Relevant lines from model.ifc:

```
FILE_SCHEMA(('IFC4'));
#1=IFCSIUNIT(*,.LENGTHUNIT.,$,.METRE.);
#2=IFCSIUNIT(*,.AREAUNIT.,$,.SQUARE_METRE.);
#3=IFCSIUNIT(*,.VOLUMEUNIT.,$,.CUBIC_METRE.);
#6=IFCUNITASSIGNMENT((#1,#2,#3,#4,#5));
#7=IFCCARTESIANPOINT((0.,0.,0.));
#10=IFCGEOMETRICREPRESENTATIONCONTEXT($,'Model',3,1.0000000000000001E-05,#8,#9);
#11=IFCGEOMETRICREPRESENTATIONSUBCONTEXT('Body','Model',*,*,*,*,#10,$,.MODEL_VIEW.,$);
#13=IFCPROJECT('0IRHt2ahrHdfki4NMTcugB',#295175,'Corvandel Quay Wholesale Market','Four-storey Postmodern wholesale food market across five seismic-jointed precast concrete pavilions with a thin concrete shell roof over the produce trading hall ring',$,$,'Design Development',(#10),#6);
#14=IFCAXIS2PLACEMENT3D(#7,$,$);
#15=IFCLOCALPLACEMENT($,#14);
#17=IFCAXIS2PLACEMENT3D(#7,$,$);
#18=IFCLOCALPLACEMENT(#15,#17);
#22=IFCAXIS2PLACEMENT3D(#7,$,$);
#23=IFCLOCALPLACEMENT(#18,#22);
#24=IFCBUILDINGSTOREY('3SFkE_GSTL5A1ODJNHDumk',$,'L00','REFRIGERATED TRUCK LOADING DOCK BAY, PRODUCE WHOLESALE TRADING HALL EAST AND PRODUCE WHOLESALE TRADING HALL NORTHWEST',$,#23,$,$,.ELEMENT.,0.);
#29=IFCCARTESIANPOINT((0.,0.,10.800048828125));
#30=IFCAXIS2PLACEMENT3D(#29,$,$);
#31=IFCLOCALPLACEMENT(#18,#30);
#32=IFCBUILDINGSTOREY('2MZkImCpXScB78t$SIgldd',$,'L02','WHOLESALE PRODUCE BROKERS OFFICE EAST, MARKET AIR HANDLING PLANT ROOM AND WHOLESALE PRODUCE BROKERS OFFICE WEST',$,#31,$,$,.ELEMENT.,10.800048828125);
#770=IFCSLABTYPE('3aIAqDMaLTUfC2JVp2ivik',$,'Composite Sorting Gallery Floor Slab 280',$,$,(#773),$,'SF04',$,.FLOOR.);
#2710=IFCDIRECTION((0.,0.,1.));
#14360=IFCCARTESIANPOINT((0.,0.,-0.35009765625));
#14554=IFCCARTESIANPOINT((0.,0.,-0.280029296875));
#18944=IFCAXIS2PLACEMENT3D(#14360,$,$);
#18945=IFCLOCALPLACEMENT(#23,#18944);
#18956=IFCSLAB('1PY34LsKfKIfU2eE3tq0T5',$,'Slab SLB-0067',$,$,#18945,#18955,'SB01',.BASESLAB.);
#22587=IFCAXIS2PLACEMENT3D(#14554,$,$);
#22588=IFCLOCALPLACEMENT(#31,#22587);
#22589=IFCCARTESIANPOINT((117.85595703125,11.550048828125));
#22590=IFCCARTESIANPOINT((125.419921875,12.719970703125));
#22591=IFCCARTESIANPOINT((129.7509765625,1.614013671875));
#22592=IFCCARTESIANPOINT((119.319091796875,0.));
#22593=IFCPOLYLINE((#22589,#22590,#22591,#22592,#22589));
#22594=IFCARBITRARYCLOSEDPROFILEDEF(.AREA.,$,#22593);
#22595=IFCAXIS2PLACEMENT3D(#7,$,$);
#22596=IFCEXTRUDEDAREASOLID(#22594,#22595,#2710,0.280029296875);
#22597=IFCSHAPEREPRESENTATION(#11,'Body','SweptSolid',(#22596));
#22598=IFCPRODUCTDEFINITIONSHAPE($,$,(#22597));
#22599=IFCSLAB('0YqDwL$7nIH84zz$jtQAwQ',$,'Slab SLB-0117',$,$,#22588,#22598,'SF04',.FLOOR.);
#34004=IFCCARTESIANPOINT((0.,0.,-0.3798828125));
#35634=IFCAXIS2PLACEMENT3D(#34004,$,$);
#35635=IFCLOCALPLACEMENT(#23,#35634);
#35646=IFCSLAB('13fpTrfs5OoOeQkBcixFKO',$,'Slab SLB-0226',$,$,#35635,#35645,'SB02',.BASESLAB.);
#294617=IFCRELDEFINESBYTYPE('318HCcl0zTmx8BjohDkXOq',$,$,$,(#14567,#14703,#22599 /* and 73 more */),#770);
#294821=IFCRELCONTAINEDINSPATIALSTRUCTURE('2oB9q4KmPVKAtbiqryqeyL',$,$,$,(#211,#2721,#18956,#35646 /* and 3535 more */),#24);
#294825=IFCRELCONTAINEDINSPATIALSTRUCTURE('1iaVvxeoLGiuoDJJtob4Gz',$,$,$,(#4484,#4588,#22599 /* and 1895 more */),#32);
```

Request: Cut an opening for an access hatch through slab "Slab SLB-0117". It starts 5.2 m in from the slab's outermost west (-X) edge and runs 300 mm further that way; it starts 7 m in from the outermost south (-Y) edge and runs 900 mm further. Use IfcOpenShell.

```python
import numpy as np
import ifcopenshell
import ifcopenshell.api.feature
import ifcopenshell.api.geometry
import ifcopenshell.api.root
import ifcopenshell.geom
import ifcopenshell.util.placement
import ifcopenshell.util.representation
import ifcopenshell.util.shape
import ifcopenshell.util.unit

model = ifcopenshell.open("model.ifc")
unit_scale = ifcopenshell.util.unit.calculate_unit_scale(model)
settings = ifcopenshell.geom.settings()


def volume(element):
    """Net volume in cubic metres, openings subtracted."""
    shape = ifcopenshell.geom.create_shape(settings, element)
    return ifcopenshell.util.shape.get_volume(shape.geometry)


slab = model.by_guid("0YqDwL$7nIH84zz$jtQAwQ")
before = volume(slab)

# Extent in the slab's own axes, in metres. The edges named are its -X and -Y sides.
slab_shape = ifcopenshell.geom.create_shape(settings, slab)
vertices = ifcopenshell.util.shape.get_vertices(slab_shape.geometry)
x_min, y_min, bottom = vertices.min(axis=0)
top = vertices[:, 2].max()

opening = ifcopenshell.api.root.create_entity(model, ifc_class="IfcOpeningElement", name="Access hatch opening", predefined_type="OPENING")
context = ifcopenshell.util.representation.get_context(model, "Model", "Body", "MODEL_VIEW")
width, depth = 0.3, 0.9
outline = [(0.0, 0.0), (width, 0.0), (width, depth), (0.0, depth), (0.0, 0.0)]
# Overshoot both faces by 50 mm so the cut is clean.
shape = ifcopenshell.api.geometry.add_slab_representation(
    model, context=context, depth=top - bottom + 0.1, polyline=outline
)
ifcopenshell.api.geometry.assign_representation(model, product=opening, representation=shape)

matrix = ifcopenshell.util.placement.get_local_placement(slab.ObjectPlacement)
matrix[:, 3] = matrix @ np.append(np.array([x_min + 5.2, y_min + 7, bottom - 0.05]) / unit_scale, 1.0)
ifcopenshell.api.geometry.edit_object_placement(model, product=opening, matrix=matrix, is_si=False)
ifcopenshell.api.feature.add_feature(model, feature=opening, element=slab)

after = volume(slab)

print(f"slab volume {before:.3f} -> {after:.3f} m3")

model.write("model_edited.ifc")
```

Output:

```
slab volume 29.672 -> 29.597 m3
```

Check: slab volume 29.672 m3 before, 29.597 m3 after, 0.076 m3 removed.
